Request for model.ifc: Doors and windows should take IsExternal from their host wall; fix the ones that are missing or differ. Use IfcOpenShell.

First a look at what the model holds.

```python
import ifcopenshell
import ifcopenshell.util.element

model = ifcopenshell.open("model.ifc")
print(model.schema)
seen = {}
for e in model.by_type("IfcDoor") + model.by_type("IfcWindow"):
    if not e.FillsVoids:
        continue
    host = e.FillsVoids[0].RelatingOpeningElement.VoidsElements[0].RelatingBuildingElement
    own = ifcopenshell.util.element.get_pset(e, f"Pset_{e.is_a()[3:].removesuffix('StandardCase')}Common", "IsExternal")
    wall = ifcopenshell.util.element.get_pset(host, "Pset_WallCommon", "IsExternal")
    seen[e.is_a(), own, wall] = seen.get((e.is_a(), own, wall), 0) + 1
for (cls, own, wall), count in sorted(seen.items(), key=str):
    print(count, cls, "IsExternal:", own, "| host wall:", wall)
```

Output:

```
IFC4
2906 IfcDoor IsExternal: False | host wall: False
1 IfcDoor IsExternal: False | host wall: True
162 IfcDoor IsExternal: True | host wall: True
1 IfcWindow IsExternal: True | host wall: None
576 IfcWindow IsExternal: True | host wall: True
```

```python
import ifcopenshell
import ifcopenshell.api.pset
import ifcopenshell.util.element

model = ifcopenshell.open("model.ifc")

count = 0
for ifc_class, pset_name in (("IfcDoor", "Pset_DoorCommon"), ("IfcWindow", "Pset_WindowCommon")):
    for e in model.by_type(ifc_class):
        if not e.FillsVoids:
            continue
        host = e.FillsVoids[0].RelatingOpeningElement.VoidsElements[0].RelatingBuildingElement
        external = ifcopenshell.util.element.get_pset(host, "Pset_WallCommon", "IsExternal")
        if external is None or ifcopenshell.util.element.get_pset(e, pset_name, "IsExternal") == external:
            continue
        pset = ifcopenshell.api.pset.add_pset(model, product=e, name=pset_name)
        ifcopenshell.api.pset.edit_pset(model, pset=pset, properties={"IsExternal": external})
        count += 1

print(count, "updated")

model.write("model_rev.ifc")
```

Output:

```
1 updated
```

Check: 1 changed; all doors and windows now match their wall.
